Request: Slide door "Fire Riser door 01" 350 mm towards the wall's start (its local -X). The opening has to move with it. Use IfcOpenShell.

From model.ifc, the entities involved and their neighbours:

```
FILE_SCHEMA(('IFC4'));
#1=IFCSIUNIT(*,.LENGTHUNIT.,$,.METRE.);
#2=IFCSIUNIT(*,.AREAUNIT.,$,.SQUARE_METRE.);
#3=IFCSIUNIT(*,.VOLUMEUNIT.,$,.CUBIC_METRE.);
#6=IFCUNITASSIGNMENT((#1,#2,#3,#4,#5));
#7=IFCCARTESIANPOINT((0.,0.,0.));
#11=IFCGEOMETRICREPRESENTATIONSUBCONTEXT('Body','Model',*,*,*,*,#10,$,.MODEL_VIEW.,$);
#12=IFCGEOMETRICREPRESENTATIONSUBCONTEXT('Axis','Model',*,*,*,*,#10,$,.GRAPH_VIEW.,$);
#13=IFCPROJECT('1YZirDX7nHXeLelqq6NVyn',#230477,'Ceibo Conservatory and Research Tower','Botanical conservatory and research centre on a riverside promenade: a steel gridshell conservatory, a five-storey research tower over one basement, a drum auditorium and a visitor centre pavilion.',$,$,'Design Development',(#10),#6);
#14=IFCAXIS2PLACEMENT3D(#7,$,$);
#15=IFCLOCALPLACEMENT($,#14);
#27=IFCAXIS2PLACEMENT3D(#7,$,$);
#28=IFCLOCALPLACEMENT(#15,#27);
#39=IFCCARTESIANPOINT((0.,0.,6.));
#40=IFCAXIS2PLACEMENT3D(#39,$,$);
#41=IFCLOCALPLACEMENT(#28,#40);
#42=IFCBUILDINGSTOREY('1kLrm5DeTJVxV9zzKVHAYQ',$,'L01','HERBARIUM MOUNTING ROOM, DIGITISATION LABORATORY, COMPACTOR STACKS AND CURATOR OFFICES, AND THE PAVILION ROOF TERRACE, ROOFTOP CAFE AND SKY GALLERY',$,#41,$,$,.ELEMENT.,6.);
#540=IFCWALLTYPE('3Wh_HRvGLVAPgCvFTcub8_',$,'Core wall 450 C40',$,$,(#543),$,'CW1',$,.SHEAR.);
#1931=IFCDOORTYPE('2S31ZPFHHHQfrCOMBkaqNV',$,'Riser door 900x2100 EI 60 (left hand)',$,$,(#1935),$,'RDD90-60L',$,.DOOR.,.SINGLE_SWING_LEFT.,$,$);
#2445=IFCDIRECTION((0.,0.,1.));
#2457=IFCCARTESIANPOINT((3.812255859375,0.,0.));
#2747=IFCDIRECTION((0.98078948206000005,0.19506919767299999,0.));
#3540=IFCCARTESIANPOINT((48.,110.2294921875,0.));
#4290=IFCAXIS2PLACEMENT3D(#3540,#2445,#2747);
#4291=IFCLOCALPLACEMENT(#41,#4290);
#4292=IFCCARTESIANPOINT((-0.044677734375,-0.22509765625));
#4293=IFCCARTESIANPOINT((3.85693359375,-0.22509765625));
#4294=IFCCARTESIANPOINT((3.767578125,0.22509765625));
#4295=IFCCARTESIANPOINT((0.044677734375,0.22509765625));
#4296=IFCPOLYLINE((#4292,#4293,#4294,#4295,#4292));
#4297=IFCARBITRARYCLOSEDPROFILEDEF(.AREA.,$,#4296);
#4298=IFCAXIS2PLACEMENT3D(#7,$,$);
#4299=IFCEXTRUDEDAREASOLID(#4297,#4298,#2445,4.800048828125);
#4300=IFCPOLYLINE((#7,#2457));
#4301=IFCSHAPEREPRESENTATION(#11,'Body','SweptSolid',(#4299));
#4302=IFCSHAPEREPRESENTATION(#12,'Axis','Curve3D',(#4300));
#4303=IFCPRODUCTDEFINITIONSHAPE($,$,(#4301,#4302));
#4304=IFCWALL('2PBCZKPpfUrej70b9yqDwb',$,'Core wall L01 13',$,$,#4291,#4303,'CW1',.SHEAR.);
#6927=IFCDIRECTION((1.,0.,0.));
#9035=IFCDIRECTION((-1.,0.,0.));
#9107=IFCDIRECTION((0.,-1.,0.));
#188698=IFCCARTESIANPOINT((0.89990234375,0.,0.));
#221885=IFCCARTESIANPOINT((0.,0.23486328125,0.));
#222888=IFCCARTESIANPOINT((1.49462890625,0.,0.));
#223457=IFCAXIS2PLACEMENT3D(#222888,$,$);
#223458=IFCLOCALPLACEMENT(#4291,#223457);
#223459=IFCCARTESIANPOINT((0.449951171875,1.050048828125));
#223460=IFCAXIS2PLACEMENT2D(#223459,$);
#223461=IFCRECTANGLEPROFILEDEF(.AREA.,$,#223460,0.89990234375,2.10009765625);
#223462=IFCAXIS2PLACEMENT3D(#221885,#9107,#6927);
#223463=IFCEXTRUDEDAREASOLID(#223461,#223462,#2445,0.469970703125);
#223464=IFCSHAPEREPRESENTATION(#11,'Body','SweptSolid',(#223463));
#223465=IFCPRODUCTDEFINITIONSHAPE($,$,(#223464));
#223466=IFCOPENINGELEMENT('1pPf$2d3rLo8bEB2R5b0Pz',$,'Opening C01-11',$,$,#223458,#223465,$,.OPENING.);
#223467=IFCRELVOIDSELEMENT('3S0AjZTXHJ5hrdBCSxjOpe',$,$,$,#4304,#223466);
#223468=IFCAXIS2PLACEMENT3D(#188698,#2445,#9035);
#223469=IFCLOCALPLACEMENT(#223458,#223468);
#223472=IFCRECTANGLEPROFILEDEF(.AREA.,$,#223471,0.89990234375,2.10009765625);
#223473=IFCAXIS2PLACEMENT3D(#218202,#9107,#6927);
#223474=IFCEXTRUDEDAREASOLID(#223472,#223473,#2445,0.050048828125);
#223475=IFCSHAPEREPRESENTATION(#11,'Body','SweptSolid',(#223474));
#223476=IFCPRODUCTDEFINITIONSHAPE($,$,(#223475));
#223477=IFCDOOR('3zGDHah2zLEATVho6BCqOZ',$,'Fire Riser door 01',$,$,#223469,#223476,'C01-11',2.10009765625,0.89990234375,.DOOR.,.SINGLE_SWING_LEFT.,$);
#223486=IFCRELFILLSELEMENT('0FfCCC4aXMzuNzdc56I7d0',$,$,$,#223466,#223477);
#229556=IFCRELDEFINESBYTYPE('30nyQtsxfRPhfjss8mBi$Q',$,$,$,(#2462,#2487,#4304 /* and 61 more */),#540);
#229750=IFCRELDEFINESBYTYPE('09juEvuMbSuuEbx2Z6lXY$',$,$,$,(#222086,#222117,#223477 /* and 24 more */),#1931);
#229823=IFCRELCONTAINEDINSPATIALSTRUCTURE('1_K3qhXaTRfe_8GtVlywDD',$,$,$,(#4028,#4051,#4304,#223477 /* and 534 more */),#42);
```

```python
import ifcopenshell
import ifcopenshell.api.geometry
import ifcopenshell.util.placement
import ifcopenshell.util.unit

model = ifcopenshell.open("model.ifc")
unit_scale = ifcopenshell.util.unit.calculate_unit_scale(model)

door = model.by_guid("3zGDHah2zLEATVho6BCqOZ")
opening = door.FillsVoids[0].RelatingOpeningElement
wall = opening.VoidsElements[0].RelatingBuildingElement

wall_matrix = ifcopenshell.util.placement.get_local_placement(wall.ObjectPlacement)
shift = wall_matrix[:3, 0] * -0.35 / unit_scale
before = ifcopenshell.util.placement.get_local_placement(door.ObjectPlacement)[:3, 3].copy()

# The door is placed relative to its opening, so it follows when the opening moves.
matrix = ifcopenshell.util.placement.get_local_placement(opening.ObjectPlacement)
matrix[:3, 3] += shift
ifcopenshell.api.geometry.edit_object_placement(
    model, product=opening, matrix=matrix, is_si=False, should_transform_children=True
)

after = ifcopenshell.util.placement.get_local_placement(door.ObjectPlacement)[:3, 3]
print("door moved by", (after - before).round(3) + 0.0)

model.write("model_v2.ifc")
```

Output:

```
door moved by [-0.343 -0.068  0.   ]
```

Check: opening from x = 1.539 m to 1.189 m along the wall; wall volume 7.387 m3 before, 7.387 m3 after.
